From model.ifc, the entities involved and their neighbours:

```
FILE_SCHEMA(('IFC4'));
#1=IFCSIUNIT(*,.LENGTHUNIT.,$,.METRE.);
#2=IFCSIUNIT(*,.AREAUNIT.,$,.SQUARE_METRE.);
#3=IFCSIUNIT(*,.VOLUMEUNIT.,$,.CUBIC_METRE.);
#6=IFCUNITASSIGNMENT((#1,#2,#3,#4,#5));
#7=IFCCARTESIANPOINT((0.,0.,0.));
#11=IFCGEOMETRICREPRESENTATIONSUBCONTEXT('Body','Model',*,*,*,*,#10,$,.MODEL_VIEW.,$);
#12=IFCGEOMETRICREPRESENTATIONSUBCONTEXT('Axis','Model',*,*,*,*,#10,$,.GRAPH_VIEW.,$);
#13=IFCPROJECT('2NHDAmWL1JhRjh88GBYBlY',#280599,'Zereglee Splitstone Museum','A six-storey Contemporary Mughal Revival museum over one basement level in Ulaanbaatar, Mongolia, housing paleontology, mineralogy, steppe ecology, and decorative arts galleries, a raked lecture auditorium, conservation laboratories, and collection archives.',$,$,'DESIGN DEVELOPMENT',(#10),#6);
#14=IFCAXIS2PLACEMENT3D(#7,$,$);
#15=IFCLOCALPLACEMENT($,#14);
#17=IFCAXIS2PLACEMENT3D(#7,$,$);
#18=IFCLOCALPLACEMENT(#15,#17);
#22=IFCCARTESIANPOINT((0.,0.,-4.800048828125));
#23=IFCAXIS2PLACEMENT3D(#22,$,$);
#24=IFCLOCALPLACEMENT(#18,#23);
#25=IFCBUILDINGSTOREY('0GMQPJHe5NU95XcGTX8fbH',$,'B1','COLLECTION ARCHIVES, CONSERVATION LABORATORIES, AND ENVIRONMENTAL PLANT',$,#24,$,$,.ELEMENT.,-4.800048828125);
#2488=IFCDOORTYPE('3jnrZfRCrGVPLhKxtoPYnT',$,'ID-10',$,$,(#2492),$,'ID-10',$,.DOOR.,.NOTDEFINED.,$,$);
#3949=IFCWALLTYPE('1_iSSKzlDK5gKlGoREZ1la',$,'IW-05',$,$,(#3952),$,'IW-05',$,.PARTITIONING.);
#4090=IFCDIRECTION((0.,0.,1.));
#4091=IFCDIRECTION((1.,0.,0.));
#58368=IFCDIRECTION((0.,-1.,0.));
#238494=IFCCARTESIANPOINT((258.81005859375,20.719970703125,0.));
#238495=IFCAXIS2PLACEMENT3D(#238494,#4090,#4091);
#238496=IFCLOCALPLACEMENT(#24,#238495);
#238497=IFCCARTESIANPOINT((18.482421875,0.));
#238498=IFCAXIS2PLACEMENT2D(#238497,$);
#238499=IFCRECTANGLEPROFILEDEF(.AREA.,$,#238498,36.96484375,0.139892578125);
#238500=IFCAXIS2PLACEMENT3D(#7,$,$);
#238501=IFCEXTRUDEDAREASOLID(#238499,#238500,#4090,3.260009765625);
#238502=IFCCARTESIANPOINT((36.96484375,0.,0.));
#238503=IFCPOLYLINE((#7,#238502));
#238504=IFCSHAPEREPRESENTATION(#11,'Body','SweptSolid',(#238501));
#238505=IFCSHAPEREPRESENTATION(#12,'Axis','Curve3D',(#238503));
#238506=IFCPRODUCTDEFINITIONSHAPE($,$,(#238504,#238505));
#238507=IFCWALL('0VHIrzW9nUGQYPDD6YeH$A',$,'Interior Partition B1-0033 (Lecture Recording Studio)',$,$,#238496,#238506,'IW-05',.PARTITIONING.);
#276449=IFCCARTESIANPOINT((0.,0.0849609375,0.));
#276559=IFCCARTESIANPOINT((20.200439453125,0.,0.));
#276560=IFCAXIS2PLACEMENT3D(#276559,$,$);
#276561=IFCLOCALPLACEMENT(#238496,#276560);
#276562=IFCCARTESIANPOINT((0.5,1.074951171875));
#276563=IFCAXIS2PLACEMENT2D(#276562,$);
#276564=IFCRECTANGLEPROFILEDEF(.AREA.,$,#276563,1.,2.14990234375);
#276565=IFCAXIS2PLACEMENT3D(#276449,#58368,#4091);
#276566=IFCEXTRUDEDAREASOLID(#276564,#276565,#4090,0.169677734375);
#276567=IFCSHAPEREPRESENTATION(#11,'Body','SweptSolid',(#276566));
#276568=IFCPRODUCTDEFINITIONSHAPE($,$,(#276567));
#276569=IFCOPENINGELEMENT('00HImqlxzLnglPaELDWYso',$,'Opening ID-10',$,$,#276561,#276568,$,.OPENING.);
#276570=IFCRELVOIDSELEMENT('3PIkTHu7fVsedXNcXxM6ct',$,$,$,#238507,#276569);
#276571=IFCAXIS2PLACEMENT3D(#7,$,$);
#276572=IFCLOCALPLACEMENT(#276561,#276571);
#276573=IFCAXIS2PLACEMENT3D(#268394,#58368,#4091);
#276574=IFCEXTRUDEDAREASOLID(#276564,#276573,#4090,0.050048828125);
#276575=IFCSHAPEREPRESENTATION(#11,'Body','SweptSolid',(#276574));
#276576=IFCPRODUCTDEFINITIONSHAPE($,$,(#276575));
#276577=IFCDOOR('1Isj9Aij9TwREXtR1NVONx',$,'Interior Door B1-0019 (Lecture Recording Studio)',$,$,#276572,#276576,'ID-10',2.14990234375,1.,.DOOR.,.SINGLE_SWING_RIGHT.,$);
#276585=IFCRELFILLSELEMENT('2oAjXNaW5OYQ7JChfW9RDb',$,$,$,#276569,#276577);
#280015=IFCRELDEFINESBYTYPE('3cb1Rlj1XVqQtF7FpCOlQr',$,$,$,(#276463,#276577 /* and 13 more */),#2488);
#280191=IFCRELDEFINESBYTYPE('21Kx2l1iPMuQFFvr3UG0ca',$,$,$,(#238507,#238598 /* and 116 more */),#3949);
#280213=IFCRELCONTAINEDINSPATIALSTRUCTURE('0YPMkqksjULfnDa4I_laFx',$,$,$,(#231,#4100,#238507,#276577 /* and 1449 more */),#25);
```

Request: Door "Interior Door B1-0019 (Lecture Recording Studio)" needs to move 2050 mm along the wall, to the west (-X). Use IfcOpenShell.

```python
import ifcopenshell
import ifcopenshell.api.geometry
import ifcopenshell.util.placement

model = ifcopenshell.open("model.ifc")

door = model.by_id(276577)
opening = door.FillsVoids[0].RelatingOpeningElement
wall = opening.VoidsElements[0].RelatingBuildingElement

wall_matrix = ifcopenshell.util.placement.get_local_placement(wall.ObjectPlacement)
shift = wall_matrix[:3, 0] * -2.05
before = ifcopenshell.util.placement.get_local_placement(door.ObjectPlacement)[:3, 3].copy()

# The door is placed relative to its opening, so it follows when the opening moves.
matrix = ifcopenshell.util.placement.get_local_placement(opening.ObjectPlacement)
matrix[:3, 3] += shift
ifcopenshell.api.geometry.edit_object_placement(
    model, product=opening, matrix=matrix, is_si=False, should_transform_children=True
)

after = ifcopenshell.util.placement.get_local_placement(door.ObjectPlacement)[:3, 3]
print("door moved by", (after - before).round(3) + 0.0)

model.write("model_rev.ifc")
```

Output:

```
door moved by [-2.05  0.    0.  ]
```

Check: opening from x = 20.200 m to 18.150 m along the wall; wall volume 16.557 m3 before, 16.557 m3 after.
